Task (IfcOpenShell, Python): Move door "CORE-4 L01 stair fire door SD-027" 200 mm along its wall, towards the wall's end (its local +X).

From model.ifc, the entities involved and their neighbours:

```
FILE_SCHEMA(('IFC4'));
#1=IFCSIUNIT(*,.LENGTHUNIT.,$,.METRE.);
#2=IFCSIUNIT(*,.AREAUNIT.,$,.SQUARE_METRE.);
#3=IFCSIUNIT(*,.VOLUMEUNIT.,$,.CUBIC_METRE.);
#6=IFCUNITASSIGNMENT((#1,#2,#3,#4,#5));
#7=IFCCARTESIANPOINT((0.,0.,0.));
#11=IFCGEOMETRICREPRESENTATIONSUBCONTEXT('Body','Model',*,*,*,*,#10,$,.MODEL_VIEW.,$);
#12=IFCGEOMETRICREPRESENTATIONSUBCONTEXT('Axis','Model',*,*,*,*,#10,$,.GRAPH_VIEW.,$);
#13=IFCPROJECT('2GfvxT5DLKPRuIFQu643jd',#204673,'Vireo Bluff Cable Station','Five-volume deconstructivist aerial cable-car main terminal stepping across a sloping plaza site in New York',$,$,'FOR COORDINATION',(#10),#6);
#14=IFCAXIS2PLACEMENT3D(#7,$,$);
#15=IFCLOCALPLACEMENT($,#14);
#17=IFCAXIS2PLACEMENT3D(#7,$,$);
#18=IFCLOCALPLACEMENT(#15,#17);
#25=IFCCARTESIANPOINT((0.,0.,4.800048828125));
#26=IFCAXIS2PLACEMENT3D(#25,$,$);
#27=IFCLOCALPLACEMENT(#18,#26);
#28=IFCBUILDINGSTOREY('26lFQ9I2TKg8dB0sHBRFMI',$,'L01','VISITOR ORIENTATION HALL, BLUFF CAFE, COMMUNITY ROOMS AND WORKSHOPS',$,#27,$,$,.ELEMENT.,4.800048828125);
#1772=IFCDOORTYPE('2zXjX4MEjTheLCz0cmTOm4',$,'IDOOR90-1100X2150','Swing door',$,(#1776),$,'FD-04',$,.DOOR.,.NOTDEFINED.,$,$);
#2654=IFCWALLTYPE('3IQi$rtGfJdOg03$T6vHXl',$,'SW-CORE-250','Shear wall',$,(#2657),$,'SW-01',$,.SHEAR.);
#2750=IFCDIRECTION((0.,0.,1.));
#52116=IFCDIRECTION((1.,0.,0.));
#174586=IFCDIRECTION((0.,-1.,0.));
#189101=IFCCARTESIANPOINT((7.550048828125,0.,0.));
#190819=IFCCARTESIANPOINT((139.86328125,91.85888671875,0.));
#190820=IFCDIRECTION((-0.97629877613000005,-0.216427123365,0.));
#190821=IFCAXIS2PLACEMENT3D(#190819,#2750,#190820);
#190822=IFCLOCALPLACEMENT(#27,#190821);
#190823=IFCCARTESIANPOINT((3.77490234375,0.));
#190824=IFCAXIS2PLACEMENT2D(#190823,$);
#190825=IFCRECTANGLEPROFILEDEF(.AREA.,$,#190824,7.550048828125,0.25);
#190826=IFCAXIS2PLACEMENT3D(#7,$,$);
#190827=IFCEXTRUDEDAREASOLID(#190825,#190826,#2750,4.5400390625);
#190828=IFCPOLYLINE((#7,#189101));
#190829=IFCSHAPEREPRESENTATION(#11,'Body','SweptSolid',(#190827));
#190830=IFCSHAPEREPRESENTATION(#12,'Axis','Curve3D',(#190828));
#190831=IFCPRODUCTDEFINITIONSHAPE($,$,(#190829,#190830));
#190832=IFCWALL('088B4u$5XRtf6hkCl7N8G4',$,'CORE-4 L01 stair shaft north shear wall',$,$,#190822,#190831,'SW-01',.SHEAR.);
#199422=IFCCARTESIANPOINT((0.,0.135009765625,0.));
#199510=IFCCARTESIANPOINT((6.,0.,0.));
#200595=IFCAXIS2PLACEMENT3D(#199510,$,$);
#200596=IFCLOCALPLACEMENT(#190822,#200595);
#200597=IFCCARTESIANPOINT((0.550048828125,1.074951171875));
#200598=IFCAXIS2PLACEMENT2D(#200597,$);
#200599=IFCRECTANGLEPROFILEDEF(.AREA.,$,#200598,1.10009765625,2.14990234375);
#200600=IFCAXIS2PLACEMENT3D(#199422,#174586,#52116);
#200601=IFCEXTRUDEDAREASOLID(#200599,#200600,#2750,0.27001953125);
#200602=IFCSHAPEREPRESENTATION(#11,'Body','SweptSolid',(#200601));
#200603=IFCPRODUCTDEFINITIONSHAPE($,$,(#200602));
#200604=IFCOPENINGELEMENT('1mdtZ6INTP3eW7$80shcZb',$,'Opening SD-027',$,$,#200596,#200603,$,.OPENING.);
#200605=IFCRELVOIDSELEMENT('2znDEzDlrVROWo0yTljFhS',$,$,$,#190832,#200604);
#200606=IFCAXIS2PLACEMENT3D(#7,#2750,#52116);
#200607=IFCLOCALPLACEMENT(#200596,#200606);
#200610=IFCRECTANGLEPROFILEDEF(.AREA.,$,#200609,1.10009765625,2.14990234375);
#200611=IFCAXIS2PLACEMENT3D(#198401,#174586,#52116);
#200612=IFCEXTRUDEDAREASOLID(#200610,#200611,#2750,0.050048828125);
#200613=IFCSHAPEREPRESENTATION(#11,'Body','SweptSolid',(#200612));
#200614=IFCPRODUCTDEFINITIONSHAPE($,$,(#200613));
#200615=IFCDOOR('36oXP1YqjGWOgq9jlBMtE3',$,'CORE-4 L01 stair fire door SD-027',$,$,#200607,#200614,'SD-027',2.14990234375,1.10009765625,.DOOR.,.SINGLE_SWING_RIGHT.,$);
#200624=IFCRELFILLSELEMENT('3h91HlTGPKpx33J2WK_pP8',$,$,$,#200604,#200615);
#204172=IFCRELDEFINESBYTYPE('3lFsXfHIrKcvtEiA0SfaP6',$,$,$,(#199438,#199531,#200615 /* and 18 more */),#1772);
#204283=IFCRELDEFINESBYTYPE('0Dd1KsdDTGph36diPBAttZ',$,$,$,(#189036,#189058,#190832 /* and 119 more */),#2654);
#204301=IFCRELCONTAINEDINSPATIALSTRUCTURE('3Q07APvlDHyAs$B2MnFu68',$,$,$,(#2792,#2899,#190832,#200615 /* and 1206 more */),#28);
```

```python
import ifcopenshell
import ifcopenshell.api.geometry
import ifcopenshell.util.placement
import ifcopenshell.util.unit

model = ifcopenshell.open("model.ifc")
unit_scale = ifcopenshell.util.unit.calculate_unit_scale(model)

door = model.by_guid("36oXP1YqjGWOgq9jlBMtE3")
opening = door.FillsVoids[0].RelatingOpeningElement
wall = opening.VoidsElements[0].RelatingBuildingElement

wall_matrix = ifcopenshell.util.placement.get_local_placement(wall.ObjectPlacement)
shift = wall_matrix[:3, 0] * 0.2 / unit_scale
before = ifcopenshell.util.placement.get_local_placement(door.ObjectPlacement)[:3, 3].copy()

# The door is placed relative to its opening, so it follows when the opening moves.
matrix = ifcopenshell.util.placement.get_local_placement(opening.ObjectPlacement)
matrix[:3, 3] += shift
ifcopenshell.api.geometry.edit_object_placement(
    model, product=opening, matrix=matrix, is_si=False, should_transform_children=True
)

after = ifcopenshell.util.placement.get_local_placement(door.ObjectPlacement)[:3, 3]
print("door moved by", (after - before).round(3) + 0.0)

model.write("model-out.ifc")
```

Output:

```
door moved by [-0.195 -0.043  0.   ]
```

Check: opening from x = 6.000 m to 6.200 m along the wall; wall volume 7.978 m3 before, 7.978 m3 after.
